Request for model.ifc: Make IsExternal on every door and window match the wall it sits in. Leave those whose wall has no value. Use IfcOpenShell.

First a look at what the model holds.

```python
import ifcopenshell
import ifcopenshell.util.element

model = ifcopenshell.open("model.ifc")
print(model.schema)
seen = {}
for e in model.by_type("IfcDoor") + model.by_type("IfcWindow"):
    if not e.FillsVoids:
        continue
    host = e.FillsVoids[0].RelatingOpeningElement.VoidsElements[0].RelatingBuildingElement
    own = ifcopenshell.util.element.get_pset(e, f"Pset_{e.is_a()[3:].removesuffix('StandardCase')}Common", "IsExternal")
    wall = ifcopenshell.util.element.get_pset(host, "Pset_WallCommon", "IsExternal")
    seen[e.is_a(), own, wall] = seen.get((e.is_a(), own, wall), 0) + 1
for (cls, own, wall), count in sorted(seen.items(), key=str):
    print(count, cls, "IsExternal:", own, "| host wall:", wall)
```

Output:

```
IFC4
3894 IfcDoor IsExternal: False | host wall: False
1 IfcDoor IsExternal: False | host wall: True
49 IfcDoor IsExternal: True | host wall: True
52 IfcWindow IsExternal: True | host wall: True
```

```python
import ifcopenshell
import ifcopenshell.api.pset
import ifcopenshell.util.element

model = ifcopenshell.open("model.ifc")

count = 0
for ifc_class, pset_name in (("IfcDoor", "Pset_DoorCommon"), ("IfcWindow", "Pset_WindowCommon")):
    for e in model.by_type(ifc_class):
        if not e.FillsVoids:
            continue
        host = e.FillsVoids[0].RelatingOpeningElement.VoidsElements[0].RelatingBuildingElement
        external = ifcopenshell.util.element.get_pset(host, "Pset_WallCommon", "IsExternal")
        if external is None or ifcopenshell.util.element.get_pset(e, pset_name, "IsExternal") == external:
            continue
        pset = ifcopenshell.api.pset.add_pset(model, product=e, name=pset_name)
        ifcopenshell.api.pset.edit_pset(model, pset=pset, properties={"IsExternal": external})
        count += 1

print(count, "updated")

model.write("model_edited.ifc")
```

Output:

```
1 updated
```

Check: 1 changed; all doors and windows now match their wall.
